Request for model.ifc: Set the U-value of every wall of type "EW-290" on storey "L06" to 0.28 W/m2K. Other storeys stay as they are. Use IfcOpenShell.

First a look at what the model holds.

```python
import ifcopenshell
import ifcopenshell.util.element

model = ifcopenshell.open("model.ifc")
print(model.schema)
storey = next(s for s in model.by_type("IfcBuildingStorey") if s.Name == "L06")
walls = [e for e in ifcopenshell.util.element.get_decomposition(storey) if e.is_a("IfcWall")]
seen = {}
for e in walls:
    element_type = ifcopenshell.util.element.get_type(e)
    key = (element_type.Name if element_type != e and element_type else None, ifcopenshell.util.element.get_pset(e, "Pset_WallCommon", "ThermalTransmittance"))
    seen[key] = seen.get(key, 0) + 1
for (name, value), count in sorted(seen.items(), key=str):
    print(count, "x", name, "|", value)
```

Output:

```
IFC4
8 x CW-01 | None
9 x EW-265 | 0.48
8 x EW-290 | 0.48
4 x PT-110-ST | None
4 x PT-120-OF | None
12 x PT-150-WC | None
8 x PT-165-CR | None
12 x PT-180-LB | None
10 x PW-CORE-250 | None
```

```python
import ifcopenshell
import ifcopenshell.api.pset
import ifcopenshell.util.element

model = ifcopenshell.open("model.ifc")

storey = next(s for s in model.by_type("IfcBuildingStorey") if s.Name == "L06")
walls = [e for e in ifcopenshell.util.element.get_decomposition(storey) if e.is_a("IfcWall")]

count = 0
for e in walls:
    element_type = ifcopenshell.util.element.get_type(e)
    if element_type in (None, e) or element_type.Name != "EW-290":
        continue
    # add_pset returns the element's existing set when there is one.
    pset = ifcopenshell.api.pset.add_pset(model, product=e, name="Pset_WallCommon")
    ifcopenshell.api.pset.edit_pset(model, pset=pset, properties={"ThermalTransmittance": 0.28})
    count += 1

print(count, "walls updated")

model.write("model_v2.ifc")
```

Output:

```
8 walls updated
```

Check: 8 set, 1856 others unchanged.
